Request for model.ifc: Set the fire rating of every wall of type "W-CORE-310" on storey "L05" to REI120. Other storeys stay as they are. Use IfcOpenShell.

First a look at what the model holds.

```python
import ifcopenshell
import ifcopenshell.util.element

model = ifcopenshell.open("model.ifc")
print(model.schema)
storey = next(s for s in model.by_type("IfcBuildingStorey") if s.Name == "L05")
walls = [e for e in ifcopenshell.util.element.get_decomposition(storey) if e.is_a("IfcWall")]
seen = {}
for e in walls:
    element_type = ifcopenshell.util.element.get_type(e)
    key = (element_type.Name if element_type != e and element_type else None, ifcopenshell.util.element.get_pset(e, "Pset_WallCommon", "FireRating"))
    seen[key] = seen.get(key, 0) + 1
for (name, value), count in sorted(seen.items(), key=str):
    print(count, "x", name, "|", value)
```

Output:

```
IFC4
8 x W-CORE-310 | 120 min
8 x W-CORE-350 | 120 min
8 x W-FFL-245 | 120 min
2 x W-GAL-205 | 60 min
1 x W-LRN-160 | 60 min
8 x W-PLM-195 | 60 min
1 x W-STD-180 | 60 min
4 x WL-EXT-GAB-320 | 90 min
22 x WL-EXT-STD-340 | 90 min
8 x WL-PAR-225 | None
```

```python
import ifcopenshell
import ifcopenshell.api.pset
import ifcopenshell.util.element

model = ifcopenshell.open("model.ifc")

storey = next(s for s in model.by_type("IfcBuildingStorey") if s.Name == "L05")
walls = [e for e in ifcopenshell.util.element.get_decomposition(storey) if e.is_a("IfcWall")]

count = 0
for e in walls:
    element_type = ifcopenshell.util.element.get_type(e)
    if element_type in (None, e) or element_type.Name != "W-CORE-310":
        continue
    # add_pset returns the element's existing set when there is one.
    pset = ifcopenshell.api.pset.add_pset(model, product=e, name="Pset_WallCommon")
    ifcopenshell.api.pset.edit_pset(model, pset=pset, properties={"FireRating": "REI120"})
    count += 1

print(count, "walls updated")

model.write("model_updated.ifc")
```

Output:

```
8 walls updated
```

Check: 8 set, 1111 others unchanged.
